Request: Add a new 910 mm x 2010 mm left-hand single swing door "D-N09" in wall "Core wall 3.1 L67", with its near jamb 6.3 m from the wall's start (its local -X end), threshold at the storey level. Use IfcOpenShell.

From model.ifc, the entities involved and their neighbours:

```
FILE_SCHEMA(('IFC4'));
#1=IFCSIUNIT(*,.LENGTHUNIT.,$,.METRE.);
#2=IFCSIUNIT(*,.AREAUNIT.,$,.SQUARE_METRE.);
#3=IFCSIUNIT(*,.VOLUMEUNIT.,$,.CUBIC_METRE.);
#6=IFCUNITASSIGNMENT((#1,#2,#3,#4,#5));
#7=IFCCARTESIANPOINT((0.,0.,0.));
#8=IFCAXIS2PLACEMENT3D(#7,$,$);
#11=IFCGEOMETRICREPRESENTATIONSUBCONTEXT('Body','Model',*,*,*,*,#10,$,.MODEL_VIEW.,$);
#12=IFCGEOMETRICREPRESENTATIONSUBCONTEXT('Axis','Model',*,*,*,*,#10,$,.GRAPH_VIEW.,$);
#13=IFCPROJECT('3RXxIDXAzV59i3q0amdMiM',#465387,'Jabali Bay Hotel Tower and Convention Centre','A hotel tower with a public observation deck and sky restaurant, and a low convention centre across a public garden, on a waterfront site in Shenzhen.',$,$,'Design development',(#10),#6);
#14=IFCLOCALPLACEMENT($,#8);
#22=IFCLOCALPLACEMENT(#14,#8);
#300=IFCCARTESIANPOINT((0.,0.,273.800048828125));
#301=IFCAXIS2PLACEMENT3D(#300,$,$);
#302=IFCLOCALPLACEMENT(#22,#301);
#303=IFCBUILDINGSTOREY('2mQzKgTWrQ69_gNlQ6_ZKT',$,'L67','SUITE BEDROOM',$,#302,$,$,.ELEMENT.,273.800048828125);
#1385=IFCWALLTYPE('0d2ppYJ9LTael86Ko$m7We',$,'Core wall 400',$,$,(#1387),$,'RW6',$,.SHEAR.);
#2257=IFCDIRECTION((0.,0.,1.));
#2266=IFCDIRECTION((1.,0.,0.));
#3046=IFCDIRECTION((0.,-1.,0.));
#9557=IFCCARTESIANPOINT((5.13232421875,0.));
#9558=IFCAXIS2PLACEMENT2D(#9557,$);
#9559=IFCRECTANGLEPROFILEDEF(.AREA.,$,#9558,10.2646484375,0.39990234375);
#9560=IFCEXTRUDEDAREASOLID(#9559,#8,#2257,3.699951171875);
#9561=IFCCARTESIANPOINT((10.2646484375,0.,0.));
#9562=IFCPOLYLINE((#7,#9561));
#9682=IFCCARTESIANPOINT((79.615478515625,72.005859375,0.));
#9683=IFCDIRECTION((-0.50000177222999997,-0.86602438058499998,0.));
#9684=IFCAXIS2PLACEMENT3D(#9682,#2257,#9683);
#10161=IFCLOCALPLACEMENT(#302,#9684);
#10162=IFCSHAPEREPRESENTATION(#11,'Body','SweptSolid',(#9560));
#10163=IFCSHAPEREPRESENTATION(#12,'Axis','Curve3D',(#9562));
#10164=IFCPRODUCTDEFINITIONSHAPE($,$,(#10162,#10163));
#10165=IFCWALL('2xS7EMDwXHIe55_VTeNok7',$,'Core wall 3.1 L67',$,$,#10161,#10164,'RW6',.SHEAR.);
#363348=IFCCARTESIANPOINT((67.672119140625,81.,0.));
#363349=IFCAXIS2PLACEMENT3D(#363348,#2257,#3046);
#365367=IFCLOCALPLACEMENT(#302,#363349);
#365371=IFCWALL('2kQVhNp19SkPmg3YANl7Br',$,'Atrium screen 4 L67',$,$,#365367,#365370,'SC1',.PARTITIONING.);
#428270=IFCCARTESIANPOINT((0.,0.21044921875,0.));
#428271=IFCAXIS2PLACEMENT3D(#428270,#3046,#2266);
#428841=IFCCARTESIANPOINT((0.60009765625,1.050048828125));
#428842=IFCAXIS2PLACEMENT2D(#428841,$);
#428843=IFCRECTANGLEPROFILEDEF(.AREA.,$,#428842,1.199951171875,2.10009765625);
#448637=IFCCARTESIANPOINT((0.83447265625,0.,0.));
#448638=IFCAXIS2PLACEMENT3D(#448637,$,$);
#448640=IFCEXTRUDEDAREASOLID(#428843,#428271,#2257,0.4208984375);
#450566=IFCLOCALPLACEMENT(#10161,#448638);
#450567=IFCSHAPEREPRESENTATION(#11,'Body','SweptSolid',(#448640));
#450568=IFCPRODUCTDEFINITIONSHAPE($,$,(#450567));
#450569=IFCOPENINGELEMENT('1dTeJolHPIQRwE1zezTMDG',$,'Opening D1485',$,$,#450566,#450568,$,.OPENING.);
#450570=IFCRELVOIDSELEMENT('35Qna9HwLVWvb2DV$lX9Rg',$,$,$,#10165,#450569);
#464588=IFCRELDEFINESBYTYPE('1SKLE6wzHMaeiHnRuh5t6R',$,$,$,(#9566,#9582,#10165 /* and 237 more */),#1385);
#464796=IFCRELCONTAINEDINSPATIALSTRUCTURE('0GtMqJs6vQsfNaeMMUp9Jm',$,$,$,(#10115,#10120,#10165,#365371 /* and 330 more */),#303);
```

```python
import numpy as np
import ifcopenshell
import ifcopenshell.api.feature
import ifcopenshell.api.geometry
import ifcopenshell.api.root
import ifcopenshell.api.spatial
import ifcopenshell.geom
import ifcopenshell.util.element
import ifcopenshell.util.placement
import ifcopenshell.util.representation
import ifcopenshell.util.shape
import ifcopenshell.util.unit

model = ifcopenshell.open("model.ifc")
unit_scale = ifcopenshell.util.unit.calculate_unit_scale(model)
settings = ifcopenshell.geom.settings()


def volume(element):
    """Net volume in cubic metres, openings subtracted."""
    shape = ifcopenshell.geom.create_shape(settings, element)
    return ifcopenshell.util.shape.get_volume(shape.geometry)


wall = model.by_guid("2xS7EMDwXHIe55_VTeNok7")
storey = ifcopenshell.util.element.get_container(wall, ifc_class="IfcBuildingStorey")
context = ifcopenshell.util.representation.get_context(model, "Model", "Body", "MODEL_VIEW")
before = volume(wall)

width, height, from_end, sill = 0.91, 2.01, 6.3, 0.0  # metres

# The wall runs along its own X axis, and the end named is its -X end.
wall_shape = ifcopenshell.geom.create_shape(settings, wall)
x, y, z = ifcopenshell.util.shape.get_vertices(wall_shape.geometry).T
start = x.min() + from_end
face, thickness = float(y.min()), float(y.max() - y.min())
wall_matrix = ifcopenshell.util.placement.get_local_placement(wall.ObjectPlacement)
level = ifcopenshell.util.placement.get_local_placement(storey.ObjectPlacement)[2, 3]


def in_wall(x, y):
    """Placement at x, y metres in the wall's axes, at sill height."""
    matrix = wall_matrix.copy()
    matrix[:, 3] = wall_matrix @ np.array([x / unit_scale, y / unit_scale, 0.0, 1.0])
    matrix[2, 3] = level + sill / unit_scale
    return matrix


# Opening: a box that overshoots both wall faces by 50 mm.
opening = ifcopenshell.api.root.create_entity(model, ifc_class="IfcOpeningElement", predefined_type="OPENING")
box = ifcopenshell.api.geometry.add_wall_representation(
    model, context=context, length=width, height=height, thickness=thickness + 0.1
)
ifcopenshell.api.geometry.assign_representation(model, product=opening, representation=box)
ifcopenshell.api.geometry.edit_object_placement(model, product=opening, matrix=in_wall(start, face - 0.05), is_si=False)
ifcopenshell.api.feature.add_feature(model, feature=opening, element=wall)

door = ifcopenshell.api.root.create_entity(model, ifc_class="IfcDoor", name="D-N09", predefined_type="DOOR")
door.OverallWidth, door.OverallHeight = width / unit_scale, height / unit_scale
door.OperationType = "SINGLE_SWING_LEFT"
body = ifcopenshell.api.geometry.add_door_representation(
    model,
    context=context,
    overall_width=door.OverallWidth,
    overall_height=door.OverallHeight,
    operation_type="SINGLE_SWING_LEFT",
    lining_properties={"LiningDepth": thickness / unit_scale, "ThresholdDepth": thickness / unit_scale},
)
ifcopenshell.api.geometry.assign_representation(model, product=door, representation=body)
ifcopenshell.api.spatial.assign_container(model, products=[door], relating_structure=storey)
ifcopenshell.api.feature.add_filling(model, opening=opening, element=door)

# The lining spans the wall, so the door starts at the wall face.
ifcopenshell.api.geometry.edit_object_placement(model, product=door, matrix=in_wall(start, face), is_si=False)

after = volume(wall)

print(f"wall volume {before:.3f} -> {after:.3f} m3")

model.write("model_rev.ifc")
```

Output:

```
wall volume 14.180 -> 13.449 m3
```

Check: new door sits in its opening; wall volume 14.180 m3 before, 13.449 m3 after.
